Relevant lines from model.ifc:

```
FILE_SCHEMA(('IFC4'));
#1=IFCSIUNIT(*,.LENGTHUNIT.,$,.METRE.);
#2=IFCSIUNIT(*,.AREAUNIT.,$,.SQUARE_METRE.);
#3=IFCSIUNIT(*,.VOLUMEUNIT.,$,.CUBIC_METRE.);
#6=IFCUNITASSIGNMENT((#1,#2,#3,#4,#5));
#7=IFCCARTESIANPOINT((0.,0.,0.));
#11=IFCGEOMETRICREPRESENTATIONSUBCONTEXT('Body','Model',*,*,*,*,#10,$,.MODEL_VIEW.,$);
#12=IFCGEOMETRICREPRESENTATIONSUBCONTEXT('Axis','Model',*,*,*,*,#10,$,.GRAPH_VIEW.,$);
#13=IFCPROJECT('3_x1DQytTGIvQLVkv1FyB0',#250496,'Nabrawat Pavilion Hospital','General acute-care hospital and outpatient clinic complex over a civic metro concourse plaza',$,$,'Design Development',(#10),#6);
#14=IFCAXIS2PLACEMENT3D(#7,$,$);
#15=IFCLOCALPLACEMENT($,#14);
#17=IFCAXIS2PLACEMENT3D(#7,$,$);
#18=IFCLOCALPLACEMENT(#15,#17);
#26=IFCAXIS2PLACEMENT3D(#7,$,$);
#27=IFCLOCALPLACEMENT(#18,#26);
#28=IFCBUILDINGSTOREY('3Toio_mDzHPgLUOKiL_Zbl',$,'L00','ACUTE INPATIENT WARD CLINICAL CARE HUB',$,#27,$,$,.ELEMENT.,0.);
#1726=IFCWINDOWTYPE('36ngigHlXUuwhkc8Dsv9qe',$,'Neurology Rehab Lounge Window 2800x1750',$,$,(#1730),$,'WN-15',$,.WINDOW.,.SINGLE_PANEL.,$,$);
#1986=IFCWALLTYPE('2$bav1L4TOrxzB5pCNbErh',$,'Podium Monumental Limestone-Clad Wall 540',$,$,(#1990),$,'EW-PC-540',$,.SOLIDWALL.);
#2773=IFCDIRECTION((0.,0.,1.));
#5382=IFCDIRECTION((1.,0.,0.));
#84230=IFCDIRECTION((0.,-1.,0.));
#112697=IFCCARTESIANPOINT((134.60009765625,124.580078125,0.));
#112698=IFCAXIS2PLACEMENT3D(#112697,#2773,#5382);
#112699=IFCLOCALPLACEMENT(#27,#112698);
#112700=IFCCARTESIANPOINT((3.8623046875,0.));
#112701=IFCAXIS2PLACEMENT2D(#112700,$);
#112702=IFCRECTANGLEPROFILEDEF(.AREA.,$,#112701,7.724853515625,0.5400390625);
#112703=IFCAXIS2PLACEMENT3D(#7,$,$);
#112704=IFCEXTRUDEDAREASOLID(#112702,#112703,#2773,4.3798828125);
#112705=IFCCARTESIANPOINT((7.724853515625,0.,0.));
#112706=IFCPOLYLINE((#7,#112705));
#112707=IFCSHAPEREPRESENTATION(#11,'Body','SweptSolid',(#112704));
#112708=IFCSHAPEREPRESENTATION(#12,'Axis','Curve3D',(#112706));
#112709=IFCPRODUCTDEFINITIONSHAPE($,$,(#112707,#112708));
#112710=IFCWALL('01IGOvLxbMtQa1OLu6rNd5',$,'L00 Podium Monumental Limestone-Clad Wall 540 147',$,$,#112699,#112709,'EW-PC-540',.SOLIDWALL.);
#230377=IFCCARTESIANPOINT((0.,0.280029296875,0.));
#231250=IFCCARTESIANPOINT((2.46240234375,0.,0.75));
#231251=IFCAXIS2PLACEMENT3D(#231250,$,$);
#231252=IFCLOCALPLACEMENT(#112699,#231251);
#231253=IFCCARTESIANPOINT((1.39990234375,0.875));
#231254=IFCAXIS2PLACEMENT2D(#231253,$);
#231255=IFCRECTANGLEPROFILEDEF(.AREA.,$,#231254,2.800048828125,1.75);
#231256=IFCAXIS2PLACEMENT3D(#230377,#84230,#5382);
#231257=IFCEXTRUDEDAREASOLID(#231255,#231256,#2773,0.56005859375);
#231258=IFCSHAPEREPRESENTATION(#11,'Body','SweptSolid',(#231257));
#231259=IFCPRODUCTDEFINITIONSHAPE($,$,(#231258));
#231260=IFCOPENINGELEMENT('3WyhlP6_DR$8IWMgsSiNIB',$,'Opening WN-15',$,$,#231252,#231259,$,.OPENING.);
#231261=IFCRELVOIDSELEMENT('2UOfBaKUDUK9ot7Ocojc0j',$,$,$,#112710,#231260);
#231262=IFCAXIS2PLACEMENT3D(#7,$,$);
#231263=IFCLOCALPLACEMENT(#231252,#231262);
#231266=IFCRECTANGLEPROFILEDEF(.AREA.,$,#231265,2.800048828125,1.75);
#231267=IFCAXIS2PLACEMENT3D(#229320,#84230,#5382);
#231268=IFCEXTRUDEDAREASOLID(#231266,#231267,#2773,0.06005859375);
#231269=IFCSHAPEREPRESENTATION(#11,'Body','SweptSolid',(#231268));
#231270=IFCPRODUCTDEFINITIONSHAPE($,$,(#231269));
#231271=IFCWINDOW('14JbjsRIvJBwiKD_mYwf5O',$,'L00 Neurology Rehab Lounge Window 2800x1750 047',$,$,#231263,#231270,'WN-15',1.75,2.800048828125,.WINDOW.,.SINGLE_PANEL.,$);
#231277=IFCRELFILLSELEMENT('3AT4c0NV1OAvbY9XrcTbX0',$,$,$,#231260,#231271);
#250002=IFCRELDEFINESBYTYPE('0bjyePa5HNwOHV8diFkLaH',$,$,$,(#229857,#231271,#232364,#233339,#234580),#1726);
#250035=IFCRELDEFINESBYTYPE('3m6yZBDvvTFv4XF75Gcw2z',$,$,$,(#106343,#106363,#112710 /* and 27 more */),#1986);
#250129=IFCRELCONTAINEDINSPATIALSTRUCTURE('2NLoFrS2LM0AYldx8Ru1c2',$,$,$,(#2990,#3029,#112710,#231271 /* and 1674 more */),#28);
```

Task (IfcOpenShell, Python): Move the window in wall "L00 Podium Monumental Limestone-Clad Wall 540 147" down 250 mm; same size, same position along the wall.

```python
import numpy as np
import ifcopenshell
import ifcopenshell.api.geometry
import ifcopenshell.util.placement
import ifcopenshell.util.unit

model = ifcopenshell.open("model.ifc")
unit_scale = ifcopenshell.util.unit.calculate_unit_scale(model)

window = model.by_guid("14JbjsRIvJBwiKD_mYwf5O")
opening = window.FillsVoids[0].RelatingOpeningElement
dz = -0.25

shift = np.array([0.0, 0.0, dz])
# The window is placed relative to its opening, so it follows when the opening moves.
matrix = ifcopenshell.util.placement.get_local_placement(opening.ObjectPlacement)
matrix[:3, 3] += shift
ifcopenshell.api.geometry.edit_object_placement(
    model, product=opening, matrix=matrix, is_si=False, should_transform_children=True
)

print(f"moved by {dz * unit_scale:+.3f} m")

model.write("model-out.ifc")
```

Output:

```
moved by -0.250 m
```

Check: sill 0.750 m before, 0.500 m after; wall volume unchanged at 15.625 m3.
